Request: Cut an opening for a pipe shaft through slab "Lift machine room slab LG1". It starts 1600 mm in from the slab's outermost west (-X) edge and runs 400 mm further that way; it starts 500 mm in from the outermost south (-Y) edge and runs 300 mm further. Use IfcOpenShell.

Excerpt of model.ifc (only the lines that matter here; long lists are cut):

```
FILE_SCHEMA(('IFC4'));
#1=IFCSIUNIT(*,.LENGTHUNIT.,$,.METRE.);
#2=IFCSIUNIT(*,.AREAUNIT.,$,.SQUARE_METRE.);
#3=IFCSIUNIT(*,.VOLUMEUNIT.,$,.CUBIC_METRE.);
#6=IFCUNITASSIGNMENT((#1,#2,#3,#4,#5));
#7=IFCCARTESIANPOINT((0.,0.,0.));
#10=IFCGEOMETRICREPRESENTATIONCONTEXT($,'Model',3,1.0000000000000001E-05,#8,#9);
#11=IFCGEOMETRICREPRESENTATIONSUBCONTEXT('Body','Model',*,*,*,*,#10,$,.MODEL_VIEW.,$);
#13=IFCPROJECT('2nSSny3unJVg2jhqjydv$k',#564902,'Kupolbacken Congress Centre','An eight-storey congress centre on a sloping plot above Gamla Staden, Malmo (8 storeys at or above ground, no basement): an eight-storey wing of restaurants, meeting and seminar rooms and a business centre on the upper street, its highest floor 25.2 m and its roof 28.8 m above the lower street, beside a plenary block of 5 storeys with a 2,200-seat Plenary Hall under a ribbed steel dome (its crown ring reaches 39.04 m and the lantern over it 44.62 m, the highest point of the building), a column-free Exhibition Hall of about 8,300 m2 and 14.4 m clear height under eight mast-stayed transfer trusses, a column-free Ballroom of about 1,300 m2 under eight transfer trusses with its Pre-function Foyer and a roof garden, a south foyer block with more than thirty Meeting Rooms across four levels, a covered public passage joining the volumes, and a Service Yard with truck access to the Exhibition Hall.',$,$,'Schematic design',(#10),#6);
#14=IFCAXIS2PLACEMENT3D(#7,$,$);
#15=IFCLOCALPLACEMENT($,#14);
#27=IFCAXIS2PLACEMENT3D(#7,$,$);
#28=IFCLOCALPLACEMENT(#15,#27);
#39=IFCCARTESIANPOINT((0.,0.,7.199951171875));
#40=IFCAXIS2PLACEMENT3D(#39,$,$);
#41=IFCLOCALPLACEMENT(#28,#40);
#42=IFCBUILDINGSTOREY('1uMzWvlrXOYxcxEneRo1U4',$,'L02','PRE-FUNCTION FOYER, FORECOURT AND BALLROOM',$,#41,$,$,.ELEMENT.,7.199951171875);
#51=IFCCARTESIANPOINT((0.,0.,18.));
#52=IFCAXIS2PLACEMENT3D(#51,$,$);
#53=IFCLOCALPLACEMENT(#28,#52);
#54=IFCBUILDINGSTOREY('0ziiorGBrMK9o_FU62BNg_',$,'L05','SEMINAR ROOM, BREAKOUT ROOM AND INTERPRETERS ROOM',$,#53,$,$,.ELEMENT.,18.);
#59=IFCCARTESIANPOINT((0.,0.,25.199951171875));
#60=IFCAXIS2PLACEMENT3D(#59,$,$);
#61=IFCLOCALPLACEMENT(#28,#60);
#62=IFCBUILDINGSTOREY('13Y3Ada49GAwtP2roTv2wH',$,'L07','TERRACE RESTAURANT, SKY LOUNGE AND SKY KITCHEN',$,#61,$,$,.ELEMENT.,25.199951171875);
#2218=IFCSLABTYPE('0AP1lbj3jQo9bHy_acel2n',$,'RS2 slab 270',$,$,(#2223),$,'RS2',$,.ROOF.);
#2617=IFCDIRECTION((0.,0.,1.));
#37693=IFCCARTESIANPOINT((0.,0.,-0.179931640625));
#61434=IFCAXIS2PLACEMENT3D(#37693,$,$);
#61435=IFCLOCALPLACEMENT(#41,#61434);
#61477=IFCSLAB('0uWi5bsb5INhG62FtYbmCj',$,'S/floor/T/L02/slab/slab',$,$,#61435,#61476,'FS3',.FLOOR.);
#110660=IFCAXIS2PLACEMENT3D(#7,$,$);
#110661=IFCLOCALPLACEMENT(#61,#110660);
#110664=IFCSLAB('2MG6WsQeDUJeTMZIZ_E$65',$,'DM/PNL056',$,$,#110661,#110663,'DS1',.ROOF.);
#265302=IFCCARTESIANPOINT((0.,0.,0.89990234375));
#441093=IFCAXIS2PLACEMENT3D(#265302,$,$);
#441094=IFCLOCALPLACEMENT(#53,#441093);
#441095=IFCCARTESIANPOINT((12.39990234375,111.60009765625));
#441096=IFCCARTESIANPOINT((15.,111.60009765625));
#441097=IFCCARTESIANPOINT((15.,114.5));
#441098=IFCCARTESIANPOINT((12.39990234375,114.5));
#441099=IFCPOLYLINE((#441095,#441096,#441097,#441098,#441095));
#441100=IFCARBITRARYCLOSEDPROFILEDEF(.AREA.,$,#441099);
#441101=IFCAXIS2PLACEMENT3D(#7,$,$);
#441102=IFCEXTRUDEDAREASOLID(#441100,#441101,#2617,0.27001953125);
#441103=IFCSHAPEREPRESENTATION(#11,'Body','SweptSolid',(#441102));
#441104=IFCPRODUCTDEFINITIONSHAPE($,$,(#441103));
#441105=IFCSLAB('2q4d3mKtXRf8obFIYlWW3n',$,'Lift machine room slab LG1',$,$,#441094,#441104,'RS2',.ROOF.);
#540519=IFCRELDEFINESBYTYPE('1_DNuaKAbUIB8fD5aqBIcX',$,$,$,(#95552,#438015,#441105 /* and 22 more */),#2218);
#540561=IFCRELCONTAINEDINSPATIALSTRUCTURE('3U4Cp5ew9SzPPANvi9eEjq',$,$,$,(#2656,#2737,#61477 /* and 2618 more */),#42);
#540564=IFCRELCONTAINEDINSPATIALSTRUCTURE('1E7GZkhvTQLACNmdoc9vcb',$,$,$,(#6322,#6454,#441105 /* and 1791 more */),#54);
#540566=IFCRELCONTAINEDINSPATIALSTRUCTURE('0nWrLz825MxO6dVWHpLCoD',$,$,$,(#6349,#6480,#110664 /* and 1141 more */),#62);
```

```python
import numpy as np
import ifcopenshell
import ifcopenshell.api.feature
import ifcopenshell.api.geometry
import ifcopenshell.api.root
import ifcopenshell.geom
import ifcopenshell.util.placement
import ifcopenshell.util.representation
import ifcopenshell.util.shape
import ifcopenshell.util.unit

model = ifcopenshell.open("model.ifc")
unit_scale = ifcopenshell.util.unit.calculate_unit_scale(model)
settings = ifcopenshell.geom.settings()


def volume(element):
    """Net volume in cubic metres, openings subtracted."""
    shape = ifcopenshell.geom.create_shape(settings, element)
    return ifcopenshell.util.shape.get_volume(shape.geometry)


slab = model.by_id(441105)
before = volume(slab)

# Extent in the slab's own axes, in metres. The edges named are its -X and -Y sides.
slab_shape = ifcopenshell.geom.create_shape(settings, slab)
vertices = ifcopenshell.util.shape.get_vertices(slab_shape.geometry)
x_min, y_min, bottom = vertices.min(axis=0)
top = vertices[:, 2].max()

opening = ifcopenshell.api.root.create_entity(model, ifc_class="IfcOpeningElement", name="Pipe shaft opening", predefined_type="OPENING")
context = ifcopenshell.util.representation.get_context(model, "Model", "Body", "MODEL_VIEW")
width, depth = 0.4, 0.3
outline = [(0.0, 0.0), (width, 0.0), (width, depth), (0.0, depth), (0.0, 0.0)]
# Overshoot both faces by 50 mm so the cut is clean.
shape = ifcopenshell.api.geometry.add_slab_representation(
    model, context=context, depth=top - bottom + 0.1, polyline=outline
)
ifcopenshell.api.geometry.assign_representation(model, product=opening, representation=shape)

matrix = ifcopenshell.util.placement.get_local_placement(slab.ObjectPlacement)
matrix[:, 3] = matrix @ np.append(np.array([x_min + 1.6, y_min + 0.5, bottom - 0.05]) / unit_scale, 1.0)
ifcopenshell.api.geometry.edit_object_placement(model, product=opening, matrix=matrix, is_si=False)
ifcopenshell.api.feature.add_feature(model, feature=opening, element=slab)

after = volume(slab)

print(f"slab volume {before:.3f} -> {after:.3f} m3")

model.write("model_updated.ifc")
```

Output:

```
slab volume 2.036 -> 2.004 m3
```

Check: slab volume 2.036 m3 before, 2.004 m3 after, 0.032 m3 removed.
